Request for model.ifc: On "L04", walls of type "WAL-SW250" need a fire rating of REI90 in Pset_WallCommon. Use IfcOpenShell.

First a look at what the model holds.

```python
import ifcopenshell
import ifcopenshell.util.element

model = ifcopenshell.open("model.ifc")
print(model.schema)
storey = next(s for s in model.by_type("IfcBuildingStorey") if s.Name == "L04")
walls = [e for e in ifcopenshell.util.element.get_decomposition(storey) if e.is_a("IfcWall")]
seen = {}
for e in walls:
    element_type = ifcopenshell.util.element.get_type(e)
    key = (element_type.Name if element_type != e and element_type else None, ifcopenshell.util.element.get_pset(e, "Pset_WallCommon", "FireRating"))
    seen[key] = seen.get(key, 0) + 1
for (name, value), count in sorted(seen.items(), key=str):
    print(count, "x", name, "|", value)
```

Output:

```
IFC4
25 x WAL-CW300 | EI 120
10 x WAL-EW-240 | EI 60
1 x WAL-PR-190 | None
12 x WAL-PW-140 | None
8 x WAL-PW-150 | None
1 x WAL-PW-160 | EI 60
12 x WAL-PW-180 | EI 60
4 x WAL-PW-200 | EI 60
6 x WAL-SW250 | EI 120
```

```python
import ifcopenshell
import ifcopenshell.api.pset
import ifcopenshell.util.element

model = ifcopenshell.open("model.ifc")

storey = next(s for s in model.by_type("IfcBuildingStorey") if s.Name == "L04")
walls = [e for e in ifcopenshell.util.element.get_decomposition(storey) if e.is_a("IfcWall")]

count = 0
for e in walls:
    element_type = ifcopenshell.util.element.get_type(e)
    if element_type in (None, e) or element_type.Name != "WAL-SW250":
        continue
    # add_pset returns the element's existing set when there is one.
    pset = ifcopenshell.api.pset.add_pset(model, product=e, name="Pset_WallCommon")
    ifcopenshell.api.pset.edit_pset(model, pset=pset, properties={"FireRating": "REI90"})
    count += 1

print(count, "walls updated")

model.write("model_v2.ifc")
```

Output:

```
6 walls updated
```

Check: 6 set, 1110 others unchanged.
